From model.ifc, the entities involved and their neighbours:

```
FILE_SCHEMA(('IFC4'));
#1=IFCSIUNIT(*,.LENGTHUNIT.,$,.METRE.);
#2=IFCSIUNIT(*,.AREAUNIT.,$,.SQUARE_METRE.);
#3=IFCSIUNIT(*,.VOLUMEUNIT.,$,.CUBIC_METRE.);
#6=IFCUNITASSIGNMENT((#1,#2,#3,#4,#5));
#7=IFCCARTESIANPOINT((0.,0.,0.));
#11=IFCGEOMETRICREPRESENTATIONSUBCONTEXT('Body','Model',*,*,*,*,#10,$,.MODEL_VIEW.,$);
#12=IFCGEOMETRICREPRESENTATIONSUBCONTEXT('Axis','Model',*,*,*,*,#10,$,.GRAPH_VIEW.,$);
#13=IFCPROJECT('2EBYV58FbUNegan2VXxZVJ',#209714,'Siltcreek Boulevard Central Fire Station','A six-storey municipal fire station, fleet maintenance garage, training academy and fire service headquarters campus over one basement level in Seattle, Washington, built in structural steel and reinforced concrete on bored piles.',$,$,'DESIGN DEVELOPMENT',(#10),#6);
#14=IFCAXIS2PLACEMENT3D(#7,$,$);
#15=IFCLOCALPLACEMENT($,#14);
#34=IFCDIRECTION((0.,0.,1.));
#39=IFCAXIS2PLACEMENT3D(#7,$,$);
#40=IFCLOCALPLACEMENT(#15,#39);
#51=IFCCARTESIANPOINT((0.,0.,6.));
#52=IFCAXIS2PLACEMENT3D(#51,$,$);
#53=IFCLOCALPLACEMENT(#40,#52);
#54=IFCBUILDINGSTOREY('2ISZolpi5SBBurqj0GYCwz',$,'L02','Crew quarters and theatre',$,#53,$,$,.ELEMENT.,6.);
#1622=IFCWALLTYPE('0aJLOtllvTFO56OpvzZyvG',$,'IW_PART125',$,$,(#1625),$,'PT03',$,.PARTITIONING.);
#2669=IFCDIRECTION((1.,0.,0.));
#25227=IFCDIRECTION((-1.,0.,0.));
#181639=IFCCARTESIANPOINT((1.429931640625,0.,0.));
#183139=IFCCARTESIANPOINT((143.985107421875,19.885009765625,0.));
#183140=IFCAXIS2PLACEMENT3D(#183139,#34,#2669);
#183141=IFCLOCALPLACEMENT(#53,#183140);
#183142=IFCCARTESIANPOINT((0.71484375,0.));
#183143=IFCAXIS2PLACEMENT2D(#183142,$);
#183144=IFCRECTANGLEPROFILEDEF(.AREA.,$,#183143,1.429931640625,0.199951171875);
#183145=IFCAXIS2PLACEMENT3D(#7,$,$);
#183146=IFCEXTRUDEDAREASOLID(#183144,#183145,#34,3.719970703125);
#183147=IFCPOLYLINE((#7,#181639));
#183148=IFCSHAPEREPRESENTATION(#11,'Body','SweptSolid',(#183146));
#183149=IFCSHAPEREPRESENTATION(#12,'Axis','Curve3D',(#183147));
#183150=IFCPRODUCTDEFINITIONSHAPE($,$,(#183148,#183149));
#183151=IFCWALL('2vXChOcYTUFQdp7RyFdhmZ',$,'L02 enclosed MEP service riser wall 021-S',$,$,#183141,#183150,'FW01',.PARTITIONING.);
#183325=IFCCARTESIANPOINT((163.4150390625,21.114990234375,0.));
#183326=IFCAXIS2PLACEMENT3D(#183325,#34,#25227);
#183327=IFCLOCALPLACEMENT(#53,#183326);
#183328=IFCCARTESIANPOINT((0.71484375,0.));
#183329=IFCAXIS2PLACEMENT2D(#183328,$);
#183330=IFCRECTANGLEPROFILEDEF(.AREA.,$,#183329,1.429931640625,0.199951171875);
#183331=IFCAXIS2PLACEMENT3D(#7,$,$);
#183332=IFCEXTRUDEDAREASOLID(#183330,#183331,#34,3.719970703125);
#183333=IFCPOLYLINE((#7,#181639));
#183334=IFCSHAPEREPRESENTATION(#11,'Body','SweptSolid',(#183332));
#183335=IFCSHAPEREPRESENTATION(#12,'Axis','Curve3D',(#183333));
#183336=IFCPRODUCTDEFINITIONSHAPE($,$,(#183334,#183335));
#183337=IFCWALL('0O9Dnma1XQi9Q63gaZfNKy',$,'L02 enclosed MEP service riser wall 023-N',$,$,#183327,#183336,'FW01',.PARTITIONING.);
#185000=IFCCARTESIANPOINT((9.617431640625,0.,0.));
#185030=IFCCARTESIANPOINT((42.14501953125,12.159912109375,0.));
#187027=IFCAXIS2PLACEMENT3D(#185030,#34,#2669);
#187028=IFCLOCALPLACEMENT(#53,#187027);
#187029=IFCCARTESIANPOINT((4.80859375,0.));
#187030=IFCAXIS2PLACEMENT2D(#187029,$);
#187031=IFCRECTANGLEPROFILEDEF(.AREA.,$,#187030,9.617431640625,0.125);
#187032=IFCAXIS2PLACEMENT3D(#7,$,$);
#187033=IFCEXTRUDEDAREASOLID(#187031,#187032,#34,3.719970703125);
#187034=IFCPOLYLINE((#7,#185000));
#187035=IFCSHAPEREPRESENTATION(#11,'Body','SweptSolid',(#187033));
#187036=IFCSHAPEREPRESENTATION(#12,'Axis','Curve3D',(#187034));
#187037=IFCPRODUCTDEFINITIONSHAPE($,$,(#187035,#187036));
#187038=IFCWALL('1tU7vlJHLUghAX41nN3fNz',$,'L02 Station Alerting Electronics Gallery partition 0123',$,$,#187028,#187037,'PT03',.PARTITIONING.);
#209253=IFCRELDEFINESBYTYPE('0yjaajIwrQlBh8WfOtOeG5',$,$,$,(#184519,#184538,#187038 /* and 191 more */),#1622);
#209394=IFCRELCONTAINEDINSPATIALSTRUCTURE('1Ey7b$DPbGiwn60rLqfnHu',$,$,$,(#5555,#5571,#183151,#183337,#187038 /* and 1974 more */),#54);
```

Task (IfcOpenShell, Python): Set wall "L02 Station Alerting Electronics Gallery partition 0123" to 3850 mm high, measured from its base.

```python
import ifcopenshell
import ifcopenshell.geom
import ifcopenshell.util.representation
import ifcopenshell.util.shape
import ifcopenshell.util.unit

model = ifcopenshell.open("model.ifc")
unit_scale = ifcopenshell.util.unit.calculate_unit_scale(model)
settings = ifcopenshell.geom.settings()


def volume(element):
    """Net volume in cubic metres, openings subtracted."""
    shape = ifcopenshell.geom.create_shape(settings, element)
    return ifcopenshell.util.shape.get_volume(shape.geometry)


wall = model.by_id(187038)
before = volume(wall)

body = ifcopenshell.util.representation.get_representation(wall, "Model", "Body")
solid = body.Items[0]
old_height = solid.Depth
solid.Depth = 3.85 / unit_scale
after = volume(wall)

print(f"height {old_height:g} -> {solid.Depth:g}, volume {before:.3f} -> {after:.3f} m3")

model.write("model_v2.ifc")
```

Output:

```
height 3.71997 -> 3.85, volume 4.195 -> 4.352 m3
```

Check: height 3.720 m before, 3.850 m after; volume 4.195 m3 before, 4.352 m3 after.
